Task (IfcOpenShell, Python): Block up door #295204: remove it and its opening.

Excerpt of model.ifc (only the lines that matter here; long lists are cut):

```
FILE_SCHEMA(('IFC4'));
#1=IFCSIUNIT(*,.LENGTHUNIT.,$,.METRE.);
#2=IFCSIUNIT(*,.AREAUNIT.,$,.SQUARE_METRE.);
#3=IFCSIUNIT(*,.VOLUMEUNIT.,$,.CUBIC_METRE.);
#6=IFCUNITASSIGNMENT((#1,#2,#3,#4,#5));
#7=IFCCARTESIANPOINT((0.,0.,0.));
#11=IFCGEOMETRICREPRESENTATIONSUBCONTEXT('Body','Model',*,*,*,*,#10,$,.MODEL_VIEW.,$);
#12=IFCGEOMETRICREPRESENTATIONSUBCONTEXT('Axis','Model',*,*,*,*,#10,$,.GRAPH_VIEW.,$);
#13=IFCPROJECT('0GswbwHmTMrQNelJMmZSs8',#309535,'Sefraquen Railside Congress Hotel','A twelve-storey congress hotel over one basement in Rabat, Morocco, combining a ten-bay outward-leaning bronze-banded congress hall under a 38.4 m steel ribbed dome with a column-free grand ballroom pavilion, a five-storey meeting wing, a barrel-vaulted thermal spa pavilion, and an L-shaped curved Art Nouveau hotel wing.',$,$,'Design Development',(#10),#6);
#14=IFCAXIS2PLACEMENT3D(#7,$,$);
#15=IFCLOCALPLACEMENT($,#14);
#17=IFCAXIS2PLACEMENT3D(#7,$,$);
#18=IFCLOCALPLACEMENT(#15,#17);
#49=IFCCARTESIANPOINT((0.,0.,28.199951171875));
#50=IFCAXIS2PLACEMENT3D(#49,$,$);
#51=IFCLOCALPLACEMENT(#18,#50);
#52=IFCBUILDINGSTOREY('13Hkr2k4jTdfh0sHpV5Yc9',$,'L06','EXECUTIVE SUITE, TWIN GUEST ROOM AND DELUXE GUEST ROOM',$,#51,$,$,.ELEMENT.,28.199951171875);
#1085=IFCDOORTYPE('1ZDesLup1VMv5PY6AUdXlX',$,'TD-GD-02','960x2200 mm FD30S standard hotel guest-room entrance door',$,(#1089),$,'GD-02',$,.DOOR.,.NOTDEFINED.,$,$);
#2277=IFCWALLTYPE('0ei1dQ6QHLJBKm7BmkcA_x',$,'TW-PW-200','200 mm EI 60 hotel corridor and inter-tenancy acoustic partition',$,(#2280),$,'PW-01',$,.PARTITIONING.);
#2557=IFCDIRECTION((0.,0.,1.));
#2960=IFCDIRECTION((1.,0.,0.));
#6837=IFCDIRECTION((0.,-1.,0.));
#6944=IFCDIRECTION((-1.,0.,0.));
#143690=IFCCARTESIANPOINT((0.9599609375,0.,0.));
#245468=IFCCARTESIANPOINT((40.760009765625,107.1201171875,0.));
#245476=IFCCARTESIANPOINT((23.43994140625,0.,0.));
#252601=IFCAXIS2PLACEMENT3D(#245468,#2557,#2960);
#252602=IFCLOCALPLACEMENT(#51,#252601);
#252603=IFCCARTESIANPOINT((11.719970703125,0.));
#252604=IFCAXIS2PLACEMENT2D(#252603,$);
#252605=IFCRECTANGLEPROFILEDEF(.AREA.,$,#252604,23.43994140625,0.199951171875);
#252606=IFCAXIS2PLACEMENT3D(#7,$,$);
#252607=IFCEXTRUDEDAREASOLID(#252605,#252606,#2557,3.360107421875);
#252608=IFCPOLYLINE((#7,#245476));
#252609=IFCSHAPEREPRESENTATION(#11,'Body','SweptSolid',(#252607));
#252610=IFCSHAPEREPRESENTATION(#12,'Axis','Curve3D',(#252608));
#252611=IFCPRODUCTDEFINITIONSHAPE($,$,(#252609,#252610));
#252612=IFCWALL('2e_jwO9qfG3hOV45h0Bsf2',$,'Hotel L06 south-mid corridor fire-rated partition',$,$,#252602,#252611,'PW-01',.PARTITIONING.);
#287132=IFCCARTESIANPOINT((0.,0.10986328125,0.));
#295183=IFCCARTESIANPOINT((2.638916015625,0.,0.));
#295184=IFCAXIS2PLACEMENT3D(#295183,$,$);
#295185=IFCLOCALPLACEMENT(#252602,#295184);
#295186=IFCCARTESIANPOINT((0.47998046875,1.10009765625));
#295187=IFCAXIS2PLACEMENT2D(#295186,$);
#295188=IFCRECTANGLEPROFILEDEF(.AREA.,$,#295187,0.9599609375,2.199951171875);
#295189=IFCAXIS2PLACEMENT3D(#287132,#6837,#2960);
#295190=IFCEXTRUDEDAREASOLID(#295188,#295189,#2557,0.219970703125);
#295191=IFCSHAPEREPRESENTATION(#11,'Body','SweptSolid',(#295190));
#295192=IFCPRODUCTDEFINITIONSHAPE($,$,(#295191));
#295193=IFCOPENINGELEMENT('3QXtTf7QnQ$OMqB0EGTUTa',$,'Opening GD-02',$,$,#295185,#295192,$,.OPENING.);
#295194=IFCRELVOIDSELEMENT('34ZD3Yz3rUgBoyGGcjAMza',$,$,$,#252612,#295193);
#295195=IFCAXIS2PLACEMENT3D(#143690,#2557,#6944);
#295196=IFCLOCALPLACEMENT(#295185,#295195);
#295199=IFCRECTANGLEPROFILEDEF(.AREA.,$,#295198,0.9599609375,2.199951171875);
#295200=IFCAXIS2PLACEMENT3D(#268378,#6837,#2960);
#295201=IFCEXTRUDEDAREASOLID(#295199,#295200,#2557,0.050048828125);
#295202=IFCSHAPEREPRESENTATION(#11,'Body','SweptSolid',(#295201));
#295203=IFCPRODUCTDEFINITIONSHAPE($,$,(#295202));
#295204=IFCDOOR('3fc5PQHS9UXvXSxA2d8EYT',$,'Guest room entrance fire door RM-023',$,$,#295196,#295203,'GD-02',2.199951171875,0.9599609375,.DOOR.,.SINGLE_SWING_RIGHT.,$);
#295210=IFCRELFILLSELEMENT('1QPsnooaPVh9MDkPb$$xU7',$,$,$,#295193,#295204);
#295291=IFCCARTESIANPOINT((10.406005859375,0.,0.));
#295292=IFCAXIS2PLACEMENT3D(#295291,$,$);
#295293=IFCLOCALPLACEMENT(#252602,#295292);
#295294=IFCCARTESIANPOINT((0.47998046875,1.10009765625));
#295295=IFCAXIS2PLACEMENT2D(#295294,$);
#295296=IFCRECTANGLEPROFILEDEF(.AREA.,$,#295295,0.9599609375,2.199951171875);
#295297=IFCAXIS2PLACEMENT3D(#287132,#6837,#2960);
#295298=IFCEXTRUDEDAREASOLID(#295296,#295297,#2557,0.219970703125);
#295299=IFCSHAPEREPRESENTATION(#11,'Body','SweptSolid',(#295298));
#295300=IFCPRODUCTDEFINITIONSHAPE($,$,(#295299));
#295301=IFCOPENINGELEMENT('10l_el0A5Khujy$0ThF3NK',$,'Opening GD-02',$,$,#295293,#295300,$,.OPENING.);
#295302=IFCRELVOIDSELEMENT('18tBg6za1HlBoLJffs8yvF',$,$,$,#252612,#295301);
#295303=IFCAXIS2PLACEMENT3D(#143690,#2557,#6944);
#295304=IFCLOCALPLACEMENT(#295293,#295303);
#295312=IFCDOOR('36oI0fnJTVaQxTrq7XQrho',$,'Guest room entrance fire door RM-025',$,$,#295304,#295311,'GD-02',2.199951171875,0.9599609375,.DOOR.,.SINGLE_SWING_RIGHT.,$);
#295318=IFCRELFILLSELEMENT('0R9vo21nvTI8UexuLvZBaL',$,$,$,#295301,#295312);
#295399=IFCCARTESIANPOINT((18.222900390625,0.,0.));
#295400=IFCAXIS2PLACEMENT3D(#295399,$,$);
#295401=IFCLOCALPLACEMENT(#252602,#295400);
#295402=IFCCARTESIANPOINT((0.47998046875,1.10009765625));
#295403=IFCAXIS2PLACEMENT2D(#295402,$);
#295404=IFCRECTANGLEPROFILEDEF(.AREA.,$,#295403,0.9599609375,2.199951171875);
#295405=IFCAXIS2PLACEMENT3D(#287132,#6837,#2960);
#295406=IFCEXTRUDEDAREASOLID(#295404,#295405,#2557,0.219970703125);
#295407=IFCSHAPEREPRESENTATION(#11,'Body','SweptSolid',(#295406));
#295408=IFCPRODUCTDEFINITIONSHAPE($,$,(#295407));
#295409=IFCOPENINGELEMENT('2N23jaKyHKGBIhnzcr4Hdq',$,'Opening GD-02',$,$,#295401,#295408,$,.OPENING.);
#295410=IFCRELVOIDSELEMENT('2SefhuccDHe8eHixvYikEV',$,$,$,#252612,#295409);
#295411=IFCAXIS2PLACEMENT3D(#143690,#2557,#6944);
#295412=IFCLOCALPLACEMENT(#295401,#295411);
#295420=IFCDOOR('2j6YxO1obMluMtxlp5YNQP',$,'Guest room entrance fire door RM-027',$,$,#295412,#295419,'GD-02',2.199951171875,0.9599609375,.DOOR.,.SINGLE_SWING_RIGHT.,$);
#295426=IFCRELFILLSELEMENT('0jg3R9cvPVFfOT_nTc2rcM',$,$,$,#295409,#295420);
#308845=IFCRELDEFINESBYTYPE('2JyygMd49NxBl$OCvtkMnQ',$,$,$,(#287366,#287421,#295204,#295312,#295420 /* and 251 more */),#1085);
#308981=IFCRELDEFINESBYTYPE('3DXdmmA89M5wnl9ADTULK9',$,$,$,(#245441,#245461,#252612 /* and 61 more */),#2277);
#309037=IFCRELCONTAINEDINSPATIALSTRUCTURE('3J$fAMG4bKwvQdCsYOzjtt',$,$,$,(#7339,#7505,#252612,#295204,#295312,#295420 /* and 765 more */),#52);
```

```python
import ifcopenshell
import ifcopenshell.api.feature
import ifcopenshell.api.root
import ifcopenshell.geom
import ifcopenshell.util.shape

model = ifcopenshell.open("model.ifc")
settings = ifcopenshell.geom.settings()


def volume(element):
    """Net volume in cubic metres, openings subtracted."""
    shape = ifcopenshell.geom.create_shape(settings, element)
    return ifcopenshell.util.shape.get_volume(shape.geometry)


door = model.by_guid("3fc5PQHS9UXvXSxA2d8EYT")
opening = door.FillsVoids[0].RelatingOpeningElement
wall = opening.VoidsElements[0].RelatingBuildingElement
before = volume(wall)

ifcopenshell.api.root.remove_product(model, product=door)
ifcopenshell.api.feature.remove_feature(model, feature=opening)

after = volume(wall)

print(f"wall volume {before:.3f} -> {after:.3f} m3")

model.write("model-out.ifc")
```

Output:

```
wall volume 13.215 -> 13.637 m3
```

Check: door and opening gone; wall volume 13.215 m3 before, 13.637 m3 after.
